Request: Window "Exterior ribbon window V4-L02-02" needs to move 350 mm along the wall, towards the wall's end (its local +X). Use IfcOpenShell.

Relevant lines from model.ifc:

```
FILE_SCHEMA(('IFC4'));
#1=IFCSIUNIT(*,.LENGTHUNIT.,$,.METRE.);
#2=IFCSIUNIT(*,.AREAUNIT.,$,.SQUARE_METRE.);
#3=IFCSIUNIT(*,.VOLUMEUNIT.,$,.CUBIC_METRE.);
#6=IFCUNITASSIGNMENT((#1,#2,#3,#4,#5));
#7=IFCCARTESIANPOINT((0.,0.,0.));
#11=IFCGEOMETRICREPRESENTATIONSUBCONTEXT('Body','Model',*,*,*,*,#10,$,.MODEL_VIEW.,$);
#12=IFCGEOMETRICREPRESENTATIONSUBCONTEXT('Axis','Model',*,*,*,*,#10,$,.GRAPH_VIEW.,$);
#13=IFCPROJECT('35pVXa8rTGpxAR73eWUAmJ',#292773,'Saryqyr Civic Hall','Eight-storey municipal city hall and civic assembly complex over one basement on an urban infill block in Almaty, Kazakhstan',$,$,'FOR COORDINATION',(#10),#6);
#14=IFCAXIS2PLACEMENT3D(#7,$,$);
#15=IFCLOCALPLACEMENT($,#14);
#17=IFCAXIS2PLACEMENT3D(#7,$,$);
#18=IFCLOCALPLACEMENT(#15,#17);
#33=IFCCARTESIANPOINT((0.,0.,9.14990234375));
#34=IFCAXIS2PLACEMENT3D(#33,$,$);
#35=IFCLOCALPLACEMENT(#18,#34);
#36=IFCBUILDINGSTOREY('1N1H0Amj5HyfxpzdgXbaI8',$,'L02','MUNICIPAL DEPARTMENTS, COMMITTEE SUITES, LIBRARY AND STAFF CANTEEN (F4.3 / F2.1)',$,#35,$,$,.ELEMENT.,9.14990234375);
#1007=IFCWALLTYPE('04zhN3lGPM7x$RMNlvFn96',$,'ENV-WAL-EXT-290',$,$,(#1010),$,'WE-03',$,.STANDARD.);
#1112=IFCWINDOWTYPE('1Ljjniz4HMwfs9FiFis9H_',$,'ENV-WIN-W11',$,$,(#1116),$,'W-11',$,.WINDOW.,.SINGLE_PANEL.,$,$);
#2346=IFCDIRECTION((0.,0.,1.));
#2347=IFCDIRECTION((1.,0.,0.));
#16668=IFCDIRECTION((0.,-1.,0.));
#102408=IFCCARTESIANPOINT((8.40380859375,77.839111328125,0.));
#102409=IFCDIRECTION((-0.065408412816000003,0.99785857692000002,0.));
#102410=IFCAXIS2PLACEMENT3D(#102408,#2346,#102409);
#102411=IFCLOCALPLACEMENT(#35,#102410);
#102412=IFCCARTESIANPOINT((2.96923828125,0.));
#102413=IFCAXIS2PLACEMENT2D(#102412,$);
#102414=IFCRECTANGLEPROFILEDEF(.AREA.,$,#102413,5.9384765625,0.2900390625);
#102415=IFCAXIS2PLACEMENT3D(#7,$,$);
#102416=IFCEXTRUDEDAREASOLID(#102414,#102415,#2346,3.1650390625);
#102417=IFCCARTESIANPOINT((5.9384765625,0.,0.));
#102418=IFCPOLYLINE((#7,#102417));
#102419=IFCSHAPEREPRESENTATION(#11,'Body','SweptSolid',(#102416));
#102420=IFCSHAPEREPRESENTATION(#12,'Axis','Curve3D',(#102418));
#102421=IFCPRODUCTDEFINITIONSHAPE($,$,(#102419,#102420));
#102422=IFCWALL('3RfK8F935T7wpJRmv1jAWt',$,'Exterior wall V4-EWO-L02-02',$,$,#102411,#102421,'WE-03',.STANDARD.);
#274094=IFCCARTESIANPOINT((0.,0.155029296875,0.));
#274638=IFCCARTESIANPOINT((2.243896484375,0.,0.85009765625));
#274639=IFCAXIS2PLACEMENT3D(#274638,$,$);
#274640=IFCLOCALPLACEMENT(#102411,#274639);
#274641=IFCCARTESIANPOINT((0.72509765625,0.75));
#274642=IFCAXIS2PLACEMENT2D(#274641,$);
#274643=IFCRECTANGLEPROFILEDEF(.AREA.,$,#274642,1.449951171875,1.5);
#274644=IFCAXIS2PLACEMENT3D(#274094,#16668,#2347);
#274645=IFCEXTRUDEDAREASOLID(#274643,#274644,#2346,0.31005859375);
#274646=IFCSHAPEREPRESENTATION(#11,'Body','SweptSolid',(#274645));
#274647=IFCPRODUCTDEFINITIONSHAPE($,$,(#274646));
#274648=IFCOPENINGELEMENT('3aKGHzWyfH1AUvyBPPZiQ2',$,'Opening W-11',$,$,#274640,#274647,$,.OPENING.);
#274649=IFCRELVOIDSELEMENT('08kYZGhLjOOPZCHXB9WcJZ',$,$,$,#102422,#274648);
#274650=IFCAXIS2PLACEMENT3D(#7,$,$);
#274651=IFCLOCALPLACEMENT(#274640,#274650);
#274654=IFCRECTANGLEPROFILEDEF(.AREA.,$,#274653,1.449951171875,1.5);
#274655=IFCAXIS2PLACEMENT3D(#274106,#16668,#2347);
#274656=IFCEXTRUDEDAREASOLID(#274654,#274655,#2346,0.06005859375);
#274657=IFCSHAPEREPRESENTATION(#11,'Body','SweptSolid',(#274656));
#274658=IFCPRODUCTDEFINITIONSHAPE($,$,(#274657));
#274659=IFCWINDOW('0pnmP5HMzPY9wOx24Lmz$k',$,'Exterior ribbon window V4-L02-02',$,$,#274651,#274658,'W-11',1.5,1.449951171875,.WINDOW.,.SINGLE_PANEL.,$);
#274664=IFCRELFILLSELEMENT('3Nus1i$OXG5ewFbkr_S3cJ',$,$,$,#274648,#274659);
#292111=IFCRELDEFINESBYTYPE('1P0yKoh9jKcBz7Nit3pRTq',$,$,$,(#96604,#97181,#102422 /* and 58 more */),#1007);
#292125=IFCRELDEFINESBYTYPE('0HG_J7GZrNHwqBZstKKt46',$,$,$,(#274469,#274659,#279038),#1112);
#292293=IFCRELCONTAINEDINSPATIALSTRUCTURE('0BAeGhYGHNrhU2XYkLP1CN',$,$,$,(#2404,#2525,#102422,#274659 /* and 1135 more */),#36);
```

```python
import ifcopenshell
import ifcopenshell.api.geometry
import ifcopenshell.util.placement
import ifcopenshell.util.unit

model = ifcopenshell.open("model.ifc")
unit_scale = ifcopenshell.util.unit.calculate_unit_scale(model)

window = model.by_guid("0pnmP5HMzPY9wOx24Lmz$k")
opening = window.FillsVoids[0].RelatingOpeningElement
wall = opening.VoidsElements[0].RelatingBuildingElement

wall_matrix = ifcopenshell.util.placement.get_local_placement(wall.ObjectPlacement)
shift = wall_matrix[:3, 0] * 0.35 / unit_scale
before = ifcopenshell.util.placement.get_local_placement(window.ObjectPlacement)[:3, 3].copy()

# The window is placed relative to its opening, so it follows when the opening moves.
matrix = ifcopenshell.util.placement.get_local_placement(opening.ObjectPlacement)
matrix[:3, 3] += shift
ifcopenshell.api.geometry.edit_object_placement(
    model, product=opening, matrix=matrix, is_si=False, should_transform_children=True
)

after = ifcopenshell.util.placement.get_local_placement(window.ObjectPlacement)[:3, 3]
print("window moved by", (after - before).round(3) + 0.0)

model.write("model-out.ifc")
```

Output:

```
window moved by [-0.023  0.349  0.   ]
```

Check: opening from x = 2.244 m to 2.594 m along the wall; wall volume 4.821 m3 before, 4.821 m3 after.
